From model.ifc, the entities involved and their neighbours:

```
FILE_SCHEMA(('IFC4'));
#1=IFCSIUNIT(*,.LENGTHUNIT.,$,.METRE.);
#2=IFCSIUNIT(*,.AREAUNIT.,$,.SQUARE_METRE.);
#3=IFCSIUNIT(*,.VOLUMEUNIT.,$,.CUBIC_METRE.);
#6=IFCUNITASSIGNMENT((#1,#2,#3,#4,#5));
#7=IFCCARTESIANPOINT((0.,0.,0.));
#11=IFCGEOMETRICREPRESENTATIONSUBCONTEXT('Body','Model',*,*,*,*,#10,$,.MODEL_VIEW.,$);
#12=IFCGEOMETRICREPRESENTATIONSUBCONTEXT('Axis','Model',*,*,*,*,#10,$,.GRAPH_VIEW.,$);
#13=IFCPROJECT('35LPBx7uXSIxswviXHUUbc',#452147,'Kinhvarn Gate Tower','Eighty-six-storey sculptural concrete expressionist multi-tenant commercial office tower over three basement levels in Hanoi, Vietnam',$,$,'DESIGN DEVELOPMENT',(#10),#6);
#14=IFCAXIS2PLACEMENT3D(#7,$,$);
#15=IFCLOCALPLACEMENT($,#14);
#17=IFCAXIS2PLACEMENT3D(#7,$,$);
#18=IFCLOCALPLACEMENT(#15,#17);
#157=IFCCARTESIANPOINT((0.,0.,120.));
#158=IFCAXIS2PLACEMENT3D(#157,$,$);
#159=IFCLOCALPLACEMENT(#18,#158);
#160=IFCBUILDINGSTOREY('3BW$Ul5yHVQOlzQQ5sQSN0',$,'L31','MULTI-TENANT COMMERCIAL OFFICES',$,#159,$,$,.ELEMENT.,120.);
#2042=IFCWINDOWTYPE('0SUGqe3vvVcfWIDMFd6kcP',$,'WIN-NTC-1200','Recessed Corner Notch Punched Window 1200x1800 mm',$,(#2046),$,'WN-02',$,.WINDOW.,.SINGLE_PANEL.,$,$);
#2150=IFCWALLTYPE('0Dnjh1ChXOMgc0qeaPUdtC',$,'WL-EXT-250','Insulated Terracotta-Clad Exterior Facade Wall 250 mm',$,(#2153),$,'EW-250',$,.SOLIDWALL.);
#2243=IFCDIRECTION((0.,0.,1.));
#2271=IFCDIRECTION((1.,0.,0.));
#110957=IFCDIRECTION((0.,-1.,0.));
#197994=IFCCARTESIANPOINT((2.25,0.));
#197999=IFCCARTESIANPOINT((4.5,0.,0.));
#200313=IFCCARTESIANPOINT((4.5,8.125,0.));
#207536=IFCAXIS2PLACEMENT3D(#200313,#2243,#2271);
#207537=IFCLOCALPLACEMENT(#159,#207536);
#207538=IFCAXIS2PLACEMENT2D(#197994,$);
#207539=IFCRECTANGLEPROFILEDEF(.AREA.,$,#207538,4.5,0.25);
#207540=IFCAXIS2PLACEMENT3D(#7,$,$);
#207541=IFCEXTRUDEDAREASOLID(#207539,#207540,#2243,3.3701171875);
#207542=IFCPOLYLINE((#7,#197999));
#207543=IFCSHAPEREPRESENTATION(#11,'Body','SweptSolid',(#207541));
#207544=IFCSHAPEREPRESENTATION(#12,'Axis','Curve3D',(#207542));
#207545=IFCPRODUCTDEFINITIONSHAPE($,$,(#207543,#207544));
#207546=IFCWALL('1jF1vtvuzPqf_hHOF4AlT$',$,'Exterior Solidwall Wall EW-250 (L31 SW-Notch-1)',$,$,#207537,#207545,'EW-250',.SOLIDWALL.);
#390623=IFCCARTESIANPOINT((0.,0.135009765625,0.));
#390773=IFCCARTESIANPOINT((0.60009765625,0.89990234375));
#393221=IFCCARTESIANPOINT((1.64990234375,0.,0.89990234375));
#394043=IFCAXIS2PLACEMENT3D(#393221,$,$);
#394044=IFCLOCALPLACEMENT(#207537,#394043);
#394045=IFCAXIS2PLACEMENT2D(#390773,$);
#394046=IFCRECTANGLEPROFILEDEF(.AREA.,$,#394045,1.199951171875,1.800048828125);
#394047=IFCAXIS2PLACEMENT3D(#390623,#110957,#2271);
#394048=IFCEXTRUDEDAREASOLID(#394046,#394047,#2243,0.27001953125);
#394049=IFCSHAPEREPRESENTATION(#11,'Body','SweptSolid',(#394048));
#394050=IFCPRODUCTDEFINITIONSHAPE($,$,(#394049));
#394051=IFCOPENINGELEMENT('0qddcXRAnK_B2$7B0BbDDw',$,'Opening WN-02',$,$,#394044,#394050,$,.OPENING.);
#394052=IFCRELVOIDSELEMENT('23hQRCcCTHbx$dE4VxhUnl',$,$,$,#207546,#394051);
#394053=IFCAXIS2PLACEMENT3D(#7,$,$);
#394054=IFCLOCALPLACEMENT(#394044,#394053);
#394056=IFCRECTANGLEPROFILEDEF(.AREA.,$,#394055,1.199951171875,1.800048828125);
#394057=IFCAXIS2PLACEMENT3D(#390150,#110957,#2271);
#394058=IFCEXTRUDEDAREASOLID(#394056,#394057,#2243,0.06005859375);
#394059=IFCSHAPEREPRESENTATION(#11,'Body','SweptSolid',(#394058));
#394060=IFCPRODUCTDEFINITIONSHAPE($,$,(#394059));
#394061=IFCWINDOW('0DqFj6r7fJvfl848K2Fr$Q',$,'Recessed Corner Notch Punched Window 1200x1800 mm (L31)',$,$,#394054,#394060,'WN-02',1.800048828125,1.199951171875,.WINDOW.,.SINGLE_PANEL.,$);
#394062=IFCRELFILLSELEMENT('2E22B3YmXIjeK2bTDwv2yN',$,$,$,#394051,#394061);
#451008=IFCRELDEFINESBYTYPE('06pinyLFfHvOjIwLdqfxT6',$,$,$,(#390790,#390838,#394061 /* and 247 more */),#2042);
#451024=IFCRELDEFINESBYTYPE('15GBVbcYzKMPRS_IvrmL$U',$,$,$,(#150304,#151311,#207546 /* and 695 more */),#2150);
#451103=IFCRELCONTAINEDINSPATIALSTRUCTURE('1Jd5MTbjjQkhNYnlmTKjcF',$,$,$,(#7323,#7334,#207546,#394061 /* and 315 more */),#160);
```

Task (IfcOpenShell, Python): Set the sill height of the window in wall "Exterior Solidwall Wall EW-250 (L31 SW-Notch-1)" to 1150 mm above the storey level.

```python
import numpy as np
import ifcopenshell
import ifcopenshell.api.geometry
import ifcopenshell.geom
import ifcopenshell.util.element
import ifcopenshell.util.placement
import ifcopenshell.util.shape
import ifcopenshell.util.unit

model = ifcopenshell.open("model.ifc")
unit_scale = ifcopenshell.util.unit.calculate_unit_scale(model)

window = model.by_guid("0DqFj6r7fJvfl848K2Fr$Q")
opening = window.FillsVoids[0].RelatingOpeningElement
storey = ifcopenshell.util.element.get_container(window, ifc_class="IfcBuildingStorey")
level = ifcopenshell.util.placement.get_local_placement(storey.ObjectPlacement)[2, 3]

# The opening's origin need not be at the sill, so measure its lowest point.
shape = ifcopenshell.geom.create_shape(ifcopenshell.geom.settings(), opening)
bottom = ifcopenshell.util.shape.get_shape_bottom_elevation(shape, shape.geometry) / unit_scale
dz = level + 1.15 / unit_scale - bottom

shift = np.array([0.0, 0.0, dz])
# The window is placed relative to its opening, so it follows when the opening moves.
matrix = ifcopenshell.util.placement.get_local_placement(opening.ObjectPlacement)
matrix[:3, 3] += shift
ifcopenshell.api.geometry.edit_object_placement(
    model, product=opening, matrix=matrix, is_si=False, should_transform_children=True
)

print(f"moved by {dz * unit_scale:+.3f} m")

model.write("model_updated.ifc")
```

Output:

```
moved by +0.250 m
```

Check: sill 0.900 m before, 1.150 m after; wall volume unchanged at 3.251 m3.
